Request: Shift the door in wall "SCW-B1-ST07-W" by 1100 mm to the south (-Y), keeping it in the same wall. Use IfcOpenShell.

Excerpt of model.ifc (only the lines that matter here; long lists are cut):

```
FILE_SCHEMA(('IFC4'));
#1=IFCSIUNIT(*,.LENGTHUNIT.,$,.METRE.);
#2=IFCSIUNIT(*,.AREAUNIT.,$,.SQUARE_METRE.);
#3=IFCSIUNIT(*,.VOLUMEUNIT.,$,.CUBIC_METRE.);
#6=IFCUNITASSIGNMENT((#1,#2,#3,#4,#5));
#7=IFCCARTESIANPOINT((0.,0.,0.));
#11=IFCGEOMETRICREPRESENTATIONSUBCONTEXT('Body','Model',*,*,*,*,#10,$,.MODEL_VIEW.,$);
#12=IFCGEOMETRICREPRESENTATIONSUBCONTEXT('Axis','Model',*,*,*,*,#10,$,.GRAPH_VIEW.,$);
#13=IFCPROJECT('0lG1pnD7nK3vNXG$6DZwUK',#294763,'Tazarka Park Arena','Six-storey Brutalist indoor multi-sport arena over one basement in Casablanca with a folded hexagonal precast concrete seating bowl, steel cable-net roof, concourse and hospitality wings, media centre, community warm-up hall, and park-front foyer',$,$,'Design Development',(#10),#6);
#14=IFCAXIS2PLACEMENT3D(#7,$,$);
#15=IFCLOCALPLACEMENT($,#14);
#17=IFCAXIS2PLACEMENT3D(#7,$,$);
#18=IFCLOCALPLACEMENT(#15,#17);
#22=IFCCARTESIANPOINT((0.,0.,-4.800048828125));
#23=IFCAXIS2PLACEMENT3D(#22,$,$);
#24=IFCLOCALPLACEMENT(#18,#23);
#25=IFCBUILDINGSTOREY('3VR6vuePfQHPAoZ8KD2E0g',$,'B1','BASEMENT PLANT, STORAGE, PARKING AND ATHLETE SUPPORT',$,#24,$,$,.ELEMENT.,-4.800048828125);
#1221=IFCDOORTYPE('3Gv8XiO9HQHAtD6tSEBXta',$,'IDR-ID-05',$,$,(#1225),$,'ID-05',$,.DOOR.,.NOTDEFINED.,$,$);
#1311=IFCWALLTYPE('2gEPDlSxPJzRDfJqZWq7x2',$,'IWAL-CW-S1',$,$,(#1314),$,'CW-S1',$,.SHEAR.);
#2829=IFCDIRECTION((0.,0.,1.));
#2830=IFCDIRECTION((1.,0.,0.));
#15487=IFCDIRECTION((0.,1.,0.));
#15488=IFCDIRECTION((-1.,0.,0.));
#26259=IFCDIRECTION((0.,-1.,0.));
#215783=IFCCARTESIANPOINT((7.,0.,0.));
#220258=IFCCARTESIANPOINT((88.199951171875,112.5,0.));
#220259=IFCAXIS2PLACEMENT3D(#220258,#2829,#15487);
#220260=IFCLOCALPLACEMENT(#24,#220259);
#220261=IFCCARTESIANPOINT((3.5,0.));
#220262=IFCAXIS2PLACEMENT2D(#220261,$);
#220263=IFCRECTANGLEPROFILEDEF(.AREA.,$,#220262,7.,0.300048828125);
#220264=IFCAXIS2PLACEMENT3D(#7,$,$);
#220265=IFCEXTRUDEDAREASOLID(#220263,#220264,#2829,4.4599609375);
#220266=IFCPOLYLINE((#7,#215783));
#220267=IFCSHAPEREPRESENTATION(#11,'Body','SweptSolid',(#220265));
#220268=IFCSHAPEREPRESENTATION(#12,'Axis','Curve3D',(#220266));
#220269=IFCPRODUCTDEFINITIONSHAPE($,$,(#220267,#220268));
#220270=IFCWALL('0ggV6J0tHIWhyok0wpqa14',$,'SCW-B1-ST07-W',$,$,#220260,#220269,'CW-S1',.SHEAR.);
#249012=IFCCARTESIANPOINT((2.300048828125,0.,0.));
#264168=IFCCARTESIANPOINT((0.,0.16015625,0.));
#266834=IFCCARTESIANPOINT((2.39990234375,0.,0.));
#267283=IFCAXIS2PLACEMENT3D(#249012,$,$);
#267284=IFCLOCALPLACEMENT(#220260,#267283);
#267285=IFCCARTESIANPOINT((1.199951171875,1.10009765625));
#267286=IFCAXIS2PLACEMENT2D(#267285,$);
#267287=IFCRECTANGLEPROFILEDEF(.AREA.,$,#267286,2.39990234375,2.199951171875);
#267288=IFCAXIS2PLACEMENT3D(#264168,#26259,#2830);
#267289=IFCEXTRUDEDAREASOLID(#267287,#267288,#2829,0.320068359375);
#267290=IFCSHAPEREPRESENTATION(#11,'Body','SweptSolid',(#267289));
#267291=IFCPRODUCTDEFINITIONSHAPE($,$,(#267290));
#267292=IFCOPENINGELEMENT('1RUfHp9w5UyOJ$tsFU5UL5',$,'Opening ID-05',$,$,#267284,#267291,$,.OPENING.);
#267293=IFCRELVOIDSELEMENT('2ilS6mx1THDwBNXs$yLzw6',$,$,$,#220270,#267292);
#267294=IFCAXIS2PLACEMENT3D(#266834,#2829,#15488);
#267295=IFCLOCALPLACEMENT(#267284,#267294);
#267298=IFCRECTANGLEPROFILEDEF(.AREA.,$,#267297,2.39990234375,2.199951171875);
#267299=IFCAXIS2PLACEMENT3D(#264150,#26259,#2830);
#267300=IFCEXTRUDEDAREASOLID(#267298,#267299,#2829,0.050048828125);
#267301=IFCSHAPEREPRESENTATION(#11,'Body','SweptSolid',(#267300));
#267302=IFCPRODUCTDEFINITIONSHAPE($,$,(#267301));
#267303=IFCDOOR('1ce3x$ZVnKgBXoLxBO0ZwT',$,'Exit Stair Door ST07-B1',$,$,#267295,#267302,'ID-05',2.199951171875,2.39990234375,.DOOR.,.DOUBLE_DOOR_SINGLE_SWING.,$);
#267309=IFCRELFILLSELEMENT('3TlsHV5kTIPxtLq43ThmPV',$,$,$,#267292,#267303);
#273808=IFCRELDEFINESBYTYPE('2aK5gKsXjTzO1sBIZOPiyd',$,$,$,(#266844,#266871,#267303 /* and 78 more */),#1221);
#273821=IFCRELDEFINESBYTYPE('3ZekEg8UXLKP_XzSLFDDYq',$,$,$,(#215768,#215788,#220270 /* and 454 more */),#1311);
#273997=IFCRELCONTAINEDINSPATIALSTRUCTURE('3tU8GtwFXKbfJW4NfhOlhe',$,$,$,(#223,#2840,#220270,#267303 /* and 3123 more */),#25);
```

```python
import ifcopenshell
import ifcopenshell.api.geometry
import ifcopenshell.util.placement

model = ifcopenshell.open("model.ifc")

door = model.by_guid("1ce3x$ZVnKgBXoLxBO0ZwT")
opening = door.FillsVoids[0].RelatingOpeningElement
wall = opening.VoidsElements[0].RelatingBuildingElement

wall_matrix = ifcopenshell.util.placement.get_local_placement(wall.ObjectPlacement)
shift = wall_matrix[:3, 0] * -1.1
before = ifcopenshell.util.placement.get_local_placement(door.ObjectPlacement)[:3, 3].copy()

# The door is placed relative to its opening, so it follows when the opening moves.
matrix = ifcopenshell.util.placement.get_local_placement(opening.ObjectPlacement)
matrix[:3, 3] += shift
ifcopenshell.api.geometry.edit_object_placement(
    model, product=opening, matrix=matrix, is_si=False, should_transform_children=True
)

after = ifcopenshell.util.placement.get_local_placement(door.ObjectPlacement)[:3, 3]
print("door moved by", (after - before).round(3) + 0.0)

model.write("model-out.ifc")
```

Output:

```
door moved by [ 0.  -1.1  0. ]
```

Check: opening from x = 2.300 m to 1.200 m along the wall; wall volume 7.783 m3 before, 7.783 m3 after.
